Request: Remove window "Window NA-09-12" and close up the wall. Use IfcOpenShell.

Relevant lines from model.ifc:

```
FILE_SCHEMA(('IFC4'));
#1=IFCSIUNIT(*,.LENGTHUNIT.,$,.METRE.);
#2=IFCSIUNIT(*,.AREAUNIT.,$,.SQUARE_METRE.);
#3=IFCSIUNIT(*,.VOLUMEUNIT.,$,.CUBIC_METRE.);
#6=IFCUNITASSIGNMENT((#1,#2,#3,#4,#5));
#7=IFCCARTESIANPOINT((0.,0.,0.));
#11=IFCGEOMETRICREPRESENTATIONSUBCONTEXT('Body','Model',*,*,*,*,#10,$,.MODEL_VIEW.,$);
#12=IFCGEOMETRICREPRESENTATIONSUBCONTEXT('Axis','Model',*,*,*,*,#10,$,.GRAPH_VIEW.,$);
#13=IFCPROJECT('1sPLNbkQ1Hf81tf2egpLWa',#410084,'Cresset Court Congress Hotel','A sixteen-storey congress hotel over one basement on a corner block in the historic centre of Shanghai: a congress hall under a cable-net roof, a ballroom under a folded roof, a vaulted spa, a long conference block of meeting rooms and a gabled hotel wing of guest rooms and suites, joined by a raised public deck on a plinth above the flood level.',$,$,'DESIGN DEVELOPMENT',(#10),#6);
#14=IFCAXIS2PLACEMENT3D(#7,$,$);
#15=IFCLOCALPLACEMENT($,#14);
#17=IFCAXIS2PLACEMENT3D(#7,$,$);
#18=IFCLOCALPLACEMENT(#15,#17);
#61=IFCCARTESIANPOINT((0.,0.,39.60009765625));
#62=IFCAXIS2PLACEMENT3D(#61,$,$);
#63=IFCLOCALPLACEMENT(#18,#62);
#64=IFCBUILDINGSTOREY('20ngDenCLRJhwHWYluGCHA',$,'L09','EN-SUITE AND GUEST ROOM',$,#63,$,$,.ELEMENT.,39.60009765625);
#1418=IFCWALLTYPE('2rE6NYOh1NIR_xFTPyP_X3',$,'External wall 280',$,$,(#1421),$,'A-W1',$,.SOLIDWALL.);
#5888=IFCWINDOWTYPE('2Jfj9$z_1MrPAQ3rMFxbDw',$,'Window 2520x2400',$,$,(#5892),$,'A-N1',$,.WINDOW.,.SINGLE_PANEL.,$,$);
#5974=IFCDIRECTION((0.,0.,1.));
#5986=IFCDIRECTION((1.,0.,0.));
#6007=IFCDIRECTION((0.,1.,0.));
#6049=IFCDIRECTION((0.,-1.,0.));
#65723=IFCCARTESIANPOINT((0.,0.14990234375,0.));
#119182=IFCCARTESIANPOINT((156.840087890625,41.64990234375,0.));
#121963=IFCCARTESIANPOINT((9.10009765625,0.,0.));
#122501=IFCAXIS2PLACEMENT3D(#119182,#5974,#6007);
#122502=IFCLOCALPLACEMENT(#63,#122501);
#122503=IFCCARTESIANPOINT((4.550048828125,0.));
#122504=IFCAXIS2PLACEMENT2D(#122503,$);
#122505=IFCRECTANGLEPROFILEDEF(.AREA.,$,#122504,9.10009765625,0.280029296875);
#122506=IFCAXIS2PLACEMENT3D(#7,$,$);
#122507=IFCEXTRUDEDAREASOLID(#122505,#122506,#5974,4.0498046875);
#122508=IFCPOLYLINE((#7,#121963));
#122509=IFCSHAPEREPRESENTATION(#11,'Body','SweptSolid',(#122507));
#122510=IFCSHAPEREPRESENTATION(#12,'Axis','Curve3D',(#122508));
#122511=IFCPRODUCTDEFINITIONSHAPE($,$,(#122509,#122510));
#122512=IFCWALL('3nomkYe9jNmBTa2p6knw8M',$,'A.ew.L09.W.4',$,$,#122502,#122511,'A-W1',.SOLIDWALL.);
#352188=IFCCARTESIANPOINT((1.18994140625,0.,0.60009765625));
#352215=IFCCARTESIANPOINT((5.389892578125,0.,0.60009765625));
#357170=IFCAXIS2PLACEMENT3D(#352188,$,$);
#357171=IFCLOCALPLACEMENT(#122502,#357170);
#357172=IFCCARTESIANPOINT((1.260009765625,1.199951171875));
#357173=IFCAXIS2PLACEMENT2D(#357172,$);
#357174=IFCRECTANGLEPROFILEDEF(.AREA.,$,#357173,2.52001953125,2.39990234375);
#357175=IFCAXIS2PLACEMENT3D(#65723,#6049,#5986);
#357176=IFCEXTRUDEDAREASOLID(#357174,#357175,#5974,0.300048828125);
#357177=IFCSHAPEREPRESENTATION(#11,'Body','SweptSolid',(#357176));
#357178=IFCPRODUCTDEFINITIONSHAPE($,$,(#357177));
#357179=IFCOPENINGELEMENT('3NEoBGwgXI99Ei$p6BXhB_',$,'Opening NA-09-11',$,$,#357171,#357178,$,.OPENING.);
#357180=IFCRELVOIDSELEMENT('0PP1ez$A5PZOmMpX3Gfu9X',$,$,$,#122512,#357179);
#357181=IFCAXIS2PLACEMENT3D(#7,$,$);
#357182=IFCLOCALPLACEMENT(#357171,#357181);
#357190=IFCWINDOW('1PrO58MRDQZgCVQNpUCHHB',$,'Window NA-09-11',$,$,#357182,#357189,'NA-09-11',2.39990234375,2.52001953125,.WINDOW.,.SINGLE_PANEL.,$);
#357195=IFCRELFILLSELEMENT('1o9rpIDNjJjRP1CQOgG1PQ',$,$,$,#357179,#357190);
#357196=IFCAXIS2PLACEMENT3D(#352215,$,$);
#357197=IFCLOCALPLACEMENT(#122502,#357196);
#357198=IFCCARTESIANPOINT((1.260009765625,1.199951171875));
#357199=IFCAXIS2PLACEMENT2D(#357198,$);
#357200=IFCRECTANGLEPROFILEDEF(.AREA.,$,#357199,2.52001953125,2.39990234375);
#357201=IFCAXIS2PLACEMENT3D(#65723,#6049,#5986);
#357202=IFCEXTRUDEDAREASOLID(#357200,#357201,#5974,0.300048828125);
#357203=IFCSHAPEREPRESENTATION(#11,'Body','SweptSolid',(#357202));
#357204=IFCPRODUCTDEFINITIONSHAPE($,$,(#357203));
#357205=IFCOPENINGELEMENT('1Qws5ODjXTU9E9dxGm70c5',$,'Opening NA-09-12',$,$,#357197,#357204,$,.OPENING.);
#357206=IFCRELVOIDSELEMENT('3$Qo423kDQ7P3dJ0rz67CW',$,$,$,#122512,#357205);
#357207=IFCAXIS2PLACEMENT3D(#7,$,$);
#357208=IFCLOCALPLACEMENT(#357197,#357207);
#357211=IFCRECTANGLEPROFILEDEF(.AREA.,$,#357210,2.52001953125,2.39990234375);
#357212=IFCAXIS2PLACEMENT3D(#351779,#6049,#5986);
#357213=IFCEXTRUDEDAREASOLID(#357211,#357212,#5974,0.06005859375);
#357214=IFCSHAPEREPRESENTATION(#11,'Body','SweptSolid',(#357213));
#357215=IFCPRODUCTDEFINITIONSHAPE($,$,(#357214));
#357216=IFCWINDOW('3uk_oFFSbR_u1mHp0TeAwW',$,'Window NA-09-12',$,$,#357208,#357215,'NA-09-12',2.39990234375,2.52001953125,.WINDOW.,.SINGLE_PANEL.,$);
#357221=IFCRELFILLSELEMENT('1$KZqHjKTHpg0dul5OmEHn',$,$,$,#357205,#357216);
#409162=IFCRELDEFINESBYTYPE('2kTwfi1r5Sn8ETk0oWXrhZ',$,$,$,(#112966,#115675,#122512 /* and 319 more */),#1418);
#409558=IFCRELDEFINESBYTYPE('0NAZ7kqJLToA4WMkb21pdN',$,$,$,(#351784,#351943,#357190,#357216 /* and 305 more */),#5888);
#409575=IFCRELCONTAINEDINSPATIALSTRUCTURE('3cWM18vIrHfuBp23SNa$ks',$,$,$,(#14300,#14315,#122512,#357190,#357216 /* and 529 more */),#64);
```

```python
import ifcopenshell
import ifcopenshell.api.feature
import ifcopenshell.api.root
import ifcopenshell.geom
import ifcopenshell.util.shape

model = ifcopenshell.open("model.ifc")
settings = ifcopenshell.geom.settings()


def volume(element):
    """Net volume in cubic metres, openings subtracted."""
    shape = ifcopenshell.geom.create_shape(settings, element)
    return ifcopenshell.util.shape.get_volume(shape.geometry)


window = model.by_guid("3uk_oFFSbR_u1mHp0TeAwW")
opening = window.FillsVoids[0].RelatingOpeningElement
wall = opening.VoidsElements[0].RelatingBuildingElement
before = volume(wall)

ifcopenshell.api.root.remove_product(model, product=window)
ifcopenshell.api.feature.remove_feature(model, feature=opening)

after = volume(wall)

print(f"wall volume {before:.3f} -> {after:.3f} m3")

model.write("model_rev.ifc")
```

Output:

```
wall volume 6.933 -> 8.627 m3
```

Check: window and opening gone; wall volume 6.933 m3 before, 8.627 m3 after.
